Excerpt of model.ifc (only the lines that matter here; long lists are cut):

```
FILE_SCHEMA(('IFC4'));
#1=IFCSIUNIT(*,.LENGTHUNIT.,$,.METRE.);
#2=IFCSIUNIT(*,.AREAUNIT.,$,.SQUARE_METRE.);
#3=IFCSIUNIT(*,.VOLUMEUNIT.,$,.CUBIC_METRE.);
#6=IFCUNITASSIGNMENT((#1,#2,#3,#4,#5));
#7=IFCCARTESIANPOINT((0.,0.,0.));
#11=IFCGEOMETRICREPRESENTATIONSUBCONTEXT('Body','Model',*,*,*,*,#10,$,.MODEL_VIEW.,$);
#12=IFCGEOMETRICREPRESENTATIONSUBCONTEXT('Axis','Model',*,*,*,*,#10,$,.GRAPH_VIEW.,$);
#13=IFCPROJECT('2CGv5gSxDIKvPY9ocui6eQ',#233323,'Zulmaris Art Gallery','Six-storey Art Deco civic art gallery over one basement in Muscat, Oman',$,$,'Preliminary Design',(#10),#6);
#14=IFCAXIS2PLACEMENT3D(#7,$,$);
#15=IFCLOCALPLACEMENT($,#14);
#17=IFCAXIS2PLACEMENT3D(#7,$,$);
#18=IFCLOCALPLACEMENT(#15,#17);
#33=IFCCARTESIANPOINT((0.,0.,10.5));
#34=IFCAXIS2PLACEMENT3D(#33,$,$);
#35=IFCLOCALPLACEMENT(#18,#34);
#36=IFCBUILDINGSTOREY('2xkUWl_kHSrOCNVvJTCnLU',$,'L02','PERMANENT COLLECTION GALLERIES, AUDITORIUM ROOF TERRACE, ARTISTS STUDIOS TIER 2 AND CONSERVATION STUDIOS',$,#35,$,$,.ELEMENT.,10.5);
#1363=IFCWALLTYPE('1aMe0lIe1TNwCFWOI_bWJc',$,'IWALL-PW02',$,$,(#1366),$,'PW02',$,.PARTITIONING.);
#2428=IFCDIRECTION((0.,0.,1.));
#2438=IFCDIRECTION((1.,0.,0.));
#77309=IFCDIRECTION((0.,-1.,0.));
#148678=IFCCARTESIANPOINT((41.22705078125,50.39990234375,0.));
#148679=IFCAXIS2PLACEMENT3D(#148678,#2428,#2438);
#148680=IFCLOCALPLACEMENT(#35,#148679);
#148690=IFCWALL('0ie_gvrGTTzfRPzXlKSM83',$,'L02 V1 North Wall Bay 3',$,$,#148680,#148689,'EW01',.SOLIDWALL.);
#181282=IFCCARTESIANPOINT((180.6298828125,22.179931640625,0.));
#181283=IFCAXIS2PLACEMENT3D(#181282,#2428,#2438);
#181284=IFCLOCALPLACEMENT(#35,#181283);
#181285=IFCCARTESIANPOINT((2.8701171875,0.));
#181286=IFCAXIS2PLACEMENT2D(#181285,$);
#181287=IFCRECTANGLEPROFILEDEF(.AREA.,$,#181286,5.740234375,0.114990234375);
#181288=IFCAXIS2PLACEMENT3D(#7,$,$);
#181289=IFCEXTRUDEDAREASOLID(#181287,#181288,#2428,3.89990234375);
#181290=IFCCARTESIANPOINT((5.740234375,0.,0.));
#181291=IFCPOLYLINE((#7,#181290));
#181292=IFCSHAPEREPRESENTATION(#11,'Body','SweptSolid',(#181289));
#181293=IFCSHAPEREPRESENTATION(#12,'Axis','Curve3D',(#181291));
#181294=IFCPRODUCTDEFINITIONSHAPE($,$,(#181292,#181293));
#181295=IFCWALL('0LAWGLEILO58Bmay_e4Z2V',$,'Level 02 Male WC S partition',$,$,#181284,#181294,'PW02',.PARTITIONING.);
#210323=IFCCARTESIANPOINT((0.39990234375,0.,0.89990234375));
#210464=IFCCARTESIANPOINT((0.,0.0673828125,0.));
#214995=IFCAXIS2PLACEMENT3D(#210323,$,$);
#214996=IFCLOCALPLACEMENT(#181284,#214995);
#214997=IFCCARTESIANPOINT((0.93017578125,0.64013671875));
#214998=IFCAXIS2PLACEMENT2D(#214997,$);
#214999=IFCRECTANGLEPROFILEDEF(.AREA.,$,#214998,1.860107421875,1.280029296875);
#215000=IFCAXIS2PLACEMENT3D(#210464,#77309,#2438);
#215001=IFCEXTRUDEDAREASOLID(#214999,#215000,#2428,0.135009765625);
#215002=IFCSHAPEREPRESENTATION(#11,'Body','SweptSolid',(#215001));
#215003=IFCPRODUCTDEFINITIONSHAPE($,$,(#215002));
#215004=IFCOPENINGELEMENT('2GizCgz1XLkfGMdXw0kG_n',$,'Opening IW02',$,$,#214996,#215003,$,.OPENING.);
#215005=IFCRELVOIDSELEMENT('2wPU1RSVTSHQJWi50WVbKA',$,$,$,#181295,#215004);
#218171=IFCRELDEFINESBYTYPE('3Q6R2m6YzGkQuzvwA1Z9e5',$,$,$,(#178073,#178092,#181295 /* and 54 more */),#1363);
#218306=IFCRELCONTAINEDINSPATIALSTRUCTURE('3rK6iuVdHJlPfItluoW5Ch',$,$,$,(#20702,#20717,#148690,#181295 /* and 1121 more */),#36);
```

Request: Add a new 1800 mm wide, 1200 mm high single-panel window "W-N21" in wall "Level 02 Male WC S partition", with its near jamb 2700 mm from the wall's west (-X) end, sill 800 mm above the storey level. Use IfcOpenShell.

```python
import numpy as np
import ifcopenshell
import ifcopenshell.api.feature
import ifcopenshell.api.geometry
import ifcopenshell.api.root
import ifcopenshell.api.spatial
import ifcopenshell.geom
import ifcopenshell.util.element
import ifcopenshell.util.placement
import ifcopenshell.util.representation
import ifcopenshell.util.shape
import ifcopenshell.util.unit

model = ifcopenshell.open("model.ifc")
unit_scale = ifcopenshell.util.unit.calculate_unit_scale(model)
settings = ifcopenshell.geom.settings()


def volume(element):
    """Net volume in cubic metres, openings subtracted."""
    shape = ifcopenshell.geom.create_shape(settings, element)
    return ifcopenshell.util.shape.get_volume(shape.geometry)


wall = model.by_guid("0LAWGLEILO58Bmay_e4Z2V")
storey = ifcopenshell.util.element.get_container(wall, ifc_class="IfcBuildingStorey")
context = ifcopenshell.util.representation.get_context(model, "Model", "Body", "MODEL_VIEW")
before = volume(wall)

width, height, from_end, sill = 1.8, 1.2, 2.7, 0.8  # metres

# The wall runs along its own X axis, and the end named is its -X end.
wall_shape = ifcopenshell.geom.create_shape(settings, wall)
x, y, z = ifcopenshell.util.shape.get_vertices(wall_shape.geometry).T
start = x.min() + from_end
face, thickness = float(y.min()), float(y.max() - y.min())
wall_matrix = ifcopenshell.util.placement.get_local_placement(wall.ObjectPlacement)
level = ifcopenshell.util.placement.get_local_placement(storey.ObjectPlacement)[2, 3]


def in_wall(x, y):
    """Placement at x, y metres in the wall's axes, at sill height."""
    matrix = wall_matrix.copy()
    matrix[:, 3] = wall_matrix @ np.array([x / unit_scale, y / unit_scale, 0.0, 1.0])
    matrix[2, 3] = level + sill / unit_scale
    return matrix


# Opening: a box that overshoots both wall faces by 50 mm.
opening = ifcopenshell.api.root.create_entity(model, ifc_class="IfcOpeningElement", predefined_type="OPENING")
box = ifcopenshell.api.geometry.add_wall_representation(
    model, context=context, length=width, height=height, thickness=thickness + 0.1
)
ifcopenshell.api.geometry.assign_representation(model, product=opening, representation=box)
ifcopenshell.api.geometry.edit_object_placement(model, product=opening, matrix=in_wall(start, face - 0.05), is_si=False)
ifcopenshell.api.feature.add_feature(model, feature=opening, element=wall)

window = ifcopenshell.api.root.create_entity(model, ifc_class="IfcWindow", name="W-N21", predefined_type="WINDOW")
window.OverallWidth, window.OverallHeight = width / unit_scale, height / unit_scale
window.PartitioningType = "SINGLE_PANEL"
body = ifcopenshell.api.geometry.add_window_representation(
    model,
    context=context,
    overall_width=window.OverallWidth,
    overall_height=window.OverallHeight,
    partition_type="SINGLE_PANEL",
)
ifcopenshell.api.geometry.assign_representation(model, product=window, representation=body)
ifcopenshell.api.spatial.assign_container(model, products=[window], relating_structure=storey)
ifcopenshell.api.feature.add_filling(model, opening=opening, element=window)

# Centre the window in the wall's thickness.
ifcopenshell.api.geometry.edit_object_placement(model, product=window, matrix=in_wall(start, face), is_si=False)
window_shape = ifcopenshell.geom.create_shape(settings, window)
depth = ifcopenshell.util.shape.get_vertices(window_shape.geometry)[:, 1]
offset = face + thickness / 2 - (depth.min() + depth.max()) / 2
ifcopenshell.api.geometry.edit_object_placement(model, product=window, matrix=in_wall(start, offset), is_si=False)

after = volume(wall)

print(f"wall volume {before:.3f} -> {after:.3f} m3")

model.write("model_rev.ifc")
```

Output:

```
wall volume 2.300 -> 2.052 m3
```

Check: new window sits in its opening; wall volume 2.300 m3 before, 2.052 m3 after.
